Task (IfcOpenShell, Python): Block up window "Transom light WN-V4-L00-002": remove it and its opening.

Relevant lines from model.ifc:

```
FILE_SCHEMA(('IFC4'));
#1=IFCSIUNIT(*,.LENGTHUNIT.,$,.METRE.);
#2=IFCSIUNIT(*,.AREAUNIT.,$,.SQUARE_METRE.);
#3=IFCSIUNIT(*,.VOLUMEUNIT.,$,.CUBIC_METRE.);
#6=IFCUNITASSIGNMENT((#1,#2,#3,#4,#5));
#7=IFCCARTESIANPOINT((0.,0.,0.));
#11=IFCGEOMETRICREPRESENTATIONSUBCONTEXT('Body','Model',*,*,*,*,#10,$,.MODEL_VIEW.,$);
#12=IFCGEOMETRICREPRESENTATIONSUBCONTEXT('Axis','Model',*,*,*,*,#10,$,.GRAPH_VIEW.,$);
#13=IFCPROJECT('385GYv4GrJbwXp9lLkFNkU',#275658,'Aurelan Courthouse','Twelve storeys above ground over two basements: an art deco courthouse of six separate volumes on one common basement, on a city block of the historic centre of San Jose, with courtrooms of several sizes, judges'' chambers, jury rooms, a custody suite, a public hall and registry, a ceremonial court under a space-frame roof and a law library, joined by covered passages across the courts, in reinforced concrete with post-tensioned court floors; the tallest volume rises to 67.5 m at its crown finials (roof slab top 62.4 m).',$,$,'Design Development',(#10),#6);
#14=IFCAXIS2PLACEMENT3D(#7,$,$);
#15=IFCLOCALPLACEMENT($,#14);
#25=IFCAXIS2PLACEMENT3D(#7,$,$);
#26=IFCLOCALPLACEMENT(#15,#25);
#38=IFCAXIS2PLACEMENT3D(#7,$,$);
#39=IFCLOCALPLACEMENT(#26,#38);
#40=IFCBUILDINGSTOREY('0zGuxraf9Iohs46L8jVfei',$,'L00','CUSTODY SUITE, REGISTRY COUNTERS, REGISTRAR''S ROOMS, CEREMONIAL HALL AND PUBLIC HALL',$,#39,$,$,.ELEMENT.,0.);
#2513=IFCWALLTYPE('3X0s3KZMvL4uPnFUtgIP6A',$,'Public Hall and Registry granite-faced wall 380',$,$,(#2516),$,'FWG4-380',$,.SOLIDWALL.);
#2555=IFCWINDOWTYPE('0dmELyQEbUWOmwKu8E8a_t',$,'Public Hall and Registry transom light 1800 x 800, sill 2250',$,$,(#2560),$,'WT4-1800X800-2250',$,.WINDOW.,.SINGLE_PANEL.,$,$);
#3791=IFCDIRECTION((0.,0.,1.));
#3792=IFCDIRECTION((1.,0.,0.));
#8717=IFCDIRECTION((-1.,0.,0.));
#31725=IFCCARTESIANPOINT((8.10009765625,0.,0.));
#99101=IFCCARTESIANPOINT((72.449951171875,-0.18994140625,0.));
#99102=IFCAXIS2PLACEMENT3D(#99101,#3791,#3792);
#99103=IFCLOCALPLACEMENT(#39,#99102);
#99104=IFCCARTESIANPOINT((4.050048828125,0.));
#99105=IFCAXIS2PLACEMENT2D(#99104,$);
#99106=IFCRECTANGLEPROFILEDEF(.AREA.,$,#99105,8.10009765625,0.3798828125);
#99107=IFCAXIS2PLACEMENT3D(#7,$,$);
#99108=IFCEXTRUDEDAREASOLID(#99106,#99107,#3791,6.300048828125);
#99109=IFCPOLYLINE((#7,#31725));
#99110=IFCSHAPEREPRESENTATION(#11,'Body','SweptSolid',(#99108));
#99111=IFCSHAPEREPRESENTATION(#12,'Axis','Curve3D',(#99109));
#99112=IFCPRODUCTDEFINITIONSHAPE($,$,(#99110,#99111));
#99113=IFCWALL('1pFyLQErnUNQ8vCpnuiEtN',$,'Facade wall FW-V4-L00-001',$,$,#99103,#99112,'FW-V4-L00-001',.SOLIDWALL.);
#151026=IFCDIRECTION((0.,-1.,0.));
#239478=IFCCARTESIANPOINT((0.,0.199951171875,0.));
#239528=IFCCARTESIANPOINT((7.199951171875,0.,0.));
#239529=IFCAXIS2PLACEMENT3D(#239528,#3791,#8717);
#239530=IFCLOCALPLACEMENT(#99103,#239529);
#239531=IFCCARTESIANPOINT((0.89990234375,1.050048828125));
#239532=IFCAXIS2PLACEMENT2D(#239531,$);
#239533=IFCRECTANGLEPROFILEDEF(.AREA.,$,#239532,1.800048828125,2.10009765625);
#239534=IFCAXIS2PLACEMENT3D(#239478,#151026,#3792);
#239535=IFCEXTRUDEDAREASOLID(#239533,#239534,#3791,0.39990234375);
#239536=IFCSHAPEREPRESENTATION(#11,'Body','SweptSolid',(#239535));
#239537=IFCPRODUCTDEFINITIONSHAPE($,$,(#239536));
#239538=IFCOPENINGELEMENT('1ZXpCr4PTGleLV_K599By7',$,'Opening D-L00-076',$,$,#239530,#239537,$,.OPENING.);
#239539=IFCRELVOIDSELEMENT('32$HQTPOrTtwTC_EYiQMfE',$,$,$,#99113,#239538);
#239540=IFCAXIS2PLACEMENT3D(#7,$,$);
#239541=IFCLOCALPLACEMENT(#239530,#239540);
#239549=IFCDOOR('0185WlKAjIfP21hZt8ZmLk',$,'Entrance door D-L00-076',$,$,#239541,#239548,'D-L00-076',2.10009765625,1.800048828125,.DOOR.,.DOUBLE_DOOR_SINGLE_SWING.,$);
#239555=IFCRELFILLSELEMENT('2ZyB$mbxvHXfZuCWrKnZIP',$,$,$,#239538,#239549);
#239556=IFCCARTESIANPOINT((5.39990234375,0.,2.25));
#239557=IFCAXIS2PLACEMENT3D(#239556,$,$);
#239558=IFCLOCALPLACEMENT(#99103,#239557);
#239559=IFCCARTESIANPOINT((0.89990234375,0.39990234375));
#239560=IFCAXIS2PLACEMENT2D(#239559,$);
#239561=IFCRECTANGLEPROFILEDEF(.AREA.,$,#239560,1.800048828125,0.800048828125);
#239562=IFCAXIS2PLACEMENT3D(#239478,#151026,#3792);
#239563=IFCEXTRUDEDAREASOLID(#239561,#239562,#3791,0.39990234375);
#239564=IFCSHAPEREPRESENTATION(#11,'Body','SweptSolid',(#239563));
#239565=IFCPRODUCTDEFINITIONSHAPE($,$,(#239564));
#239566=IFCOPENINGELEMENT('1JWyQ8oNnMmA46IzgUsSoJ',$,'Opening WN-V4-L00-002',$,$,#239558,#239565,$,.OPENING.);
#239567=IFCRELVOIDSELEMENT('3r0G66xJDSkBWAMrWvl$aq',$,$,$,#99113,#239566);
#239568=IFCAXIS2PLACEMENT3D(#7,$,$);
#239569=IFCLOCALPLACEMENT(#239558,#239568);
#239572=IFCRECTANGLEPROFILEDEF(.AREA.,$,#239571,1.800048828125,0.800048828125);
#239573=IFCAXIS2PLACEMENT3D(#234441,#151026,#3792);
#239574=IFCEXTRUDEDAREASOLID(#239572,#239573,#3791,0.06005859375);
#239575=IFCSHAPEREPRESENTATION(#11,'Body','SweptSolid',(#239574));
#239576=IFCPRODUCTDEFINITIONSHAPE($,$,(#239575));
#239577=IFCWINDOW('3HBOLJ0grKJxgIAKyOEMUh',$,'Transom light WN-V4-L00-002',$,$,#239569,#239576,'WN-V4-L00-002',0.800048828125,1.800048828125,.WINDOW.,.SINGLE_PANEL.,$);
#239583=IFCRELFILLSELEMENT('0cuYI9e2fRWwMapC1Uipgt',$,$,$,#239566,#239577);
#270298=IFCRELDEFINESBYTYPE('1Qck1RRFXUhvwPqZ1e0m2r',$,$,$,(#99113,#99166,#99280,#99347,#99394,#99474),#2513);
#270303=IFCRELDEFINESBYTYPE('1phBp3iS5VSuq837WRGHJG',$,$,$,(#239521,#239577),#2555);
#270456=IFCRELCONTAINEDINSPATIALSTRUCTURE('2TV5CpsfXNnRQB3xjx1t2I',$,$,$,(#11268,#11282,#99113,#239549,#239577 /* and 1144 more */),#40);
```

```python
import ifcopenshell
import ifcopenshell.api.feature
import ifcopenshell.api.root
import ifcopenshell.geom
import ifcopenshell.util.shape

model = ifcopenshell.open("model.ifc")
settings = ifcopenshell.geom.settings()


def volume(element):
    """Net volume in cubic metres, openings subtracted."""
    shape = ifcopenshell.geom.create_shape(settings, element)
    return ifcopenshell.util.shape.get_volume(shape.geometry)


window = model.by_guid("3HBOLJ0grKJxgIAKyOEMUh")
opening = window.FillsVoids[0].RelatingOpeningElement
wall = opening.VoidsElements[0].RelatingBuildingElement
before = volume(wall)

ifcopenshell.api.root.remove_product(model, product=window)
ifcopenshell.api.feature.remove_feature(model, feature=opening)

after = volume(wall)

print(f"wall volume {before:.3f} -> {after:.3f} m3")

model.write("model_updated.ifc")
```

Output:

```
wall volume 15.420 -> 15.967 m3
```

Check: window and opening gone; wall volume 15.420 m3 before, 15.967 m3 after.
